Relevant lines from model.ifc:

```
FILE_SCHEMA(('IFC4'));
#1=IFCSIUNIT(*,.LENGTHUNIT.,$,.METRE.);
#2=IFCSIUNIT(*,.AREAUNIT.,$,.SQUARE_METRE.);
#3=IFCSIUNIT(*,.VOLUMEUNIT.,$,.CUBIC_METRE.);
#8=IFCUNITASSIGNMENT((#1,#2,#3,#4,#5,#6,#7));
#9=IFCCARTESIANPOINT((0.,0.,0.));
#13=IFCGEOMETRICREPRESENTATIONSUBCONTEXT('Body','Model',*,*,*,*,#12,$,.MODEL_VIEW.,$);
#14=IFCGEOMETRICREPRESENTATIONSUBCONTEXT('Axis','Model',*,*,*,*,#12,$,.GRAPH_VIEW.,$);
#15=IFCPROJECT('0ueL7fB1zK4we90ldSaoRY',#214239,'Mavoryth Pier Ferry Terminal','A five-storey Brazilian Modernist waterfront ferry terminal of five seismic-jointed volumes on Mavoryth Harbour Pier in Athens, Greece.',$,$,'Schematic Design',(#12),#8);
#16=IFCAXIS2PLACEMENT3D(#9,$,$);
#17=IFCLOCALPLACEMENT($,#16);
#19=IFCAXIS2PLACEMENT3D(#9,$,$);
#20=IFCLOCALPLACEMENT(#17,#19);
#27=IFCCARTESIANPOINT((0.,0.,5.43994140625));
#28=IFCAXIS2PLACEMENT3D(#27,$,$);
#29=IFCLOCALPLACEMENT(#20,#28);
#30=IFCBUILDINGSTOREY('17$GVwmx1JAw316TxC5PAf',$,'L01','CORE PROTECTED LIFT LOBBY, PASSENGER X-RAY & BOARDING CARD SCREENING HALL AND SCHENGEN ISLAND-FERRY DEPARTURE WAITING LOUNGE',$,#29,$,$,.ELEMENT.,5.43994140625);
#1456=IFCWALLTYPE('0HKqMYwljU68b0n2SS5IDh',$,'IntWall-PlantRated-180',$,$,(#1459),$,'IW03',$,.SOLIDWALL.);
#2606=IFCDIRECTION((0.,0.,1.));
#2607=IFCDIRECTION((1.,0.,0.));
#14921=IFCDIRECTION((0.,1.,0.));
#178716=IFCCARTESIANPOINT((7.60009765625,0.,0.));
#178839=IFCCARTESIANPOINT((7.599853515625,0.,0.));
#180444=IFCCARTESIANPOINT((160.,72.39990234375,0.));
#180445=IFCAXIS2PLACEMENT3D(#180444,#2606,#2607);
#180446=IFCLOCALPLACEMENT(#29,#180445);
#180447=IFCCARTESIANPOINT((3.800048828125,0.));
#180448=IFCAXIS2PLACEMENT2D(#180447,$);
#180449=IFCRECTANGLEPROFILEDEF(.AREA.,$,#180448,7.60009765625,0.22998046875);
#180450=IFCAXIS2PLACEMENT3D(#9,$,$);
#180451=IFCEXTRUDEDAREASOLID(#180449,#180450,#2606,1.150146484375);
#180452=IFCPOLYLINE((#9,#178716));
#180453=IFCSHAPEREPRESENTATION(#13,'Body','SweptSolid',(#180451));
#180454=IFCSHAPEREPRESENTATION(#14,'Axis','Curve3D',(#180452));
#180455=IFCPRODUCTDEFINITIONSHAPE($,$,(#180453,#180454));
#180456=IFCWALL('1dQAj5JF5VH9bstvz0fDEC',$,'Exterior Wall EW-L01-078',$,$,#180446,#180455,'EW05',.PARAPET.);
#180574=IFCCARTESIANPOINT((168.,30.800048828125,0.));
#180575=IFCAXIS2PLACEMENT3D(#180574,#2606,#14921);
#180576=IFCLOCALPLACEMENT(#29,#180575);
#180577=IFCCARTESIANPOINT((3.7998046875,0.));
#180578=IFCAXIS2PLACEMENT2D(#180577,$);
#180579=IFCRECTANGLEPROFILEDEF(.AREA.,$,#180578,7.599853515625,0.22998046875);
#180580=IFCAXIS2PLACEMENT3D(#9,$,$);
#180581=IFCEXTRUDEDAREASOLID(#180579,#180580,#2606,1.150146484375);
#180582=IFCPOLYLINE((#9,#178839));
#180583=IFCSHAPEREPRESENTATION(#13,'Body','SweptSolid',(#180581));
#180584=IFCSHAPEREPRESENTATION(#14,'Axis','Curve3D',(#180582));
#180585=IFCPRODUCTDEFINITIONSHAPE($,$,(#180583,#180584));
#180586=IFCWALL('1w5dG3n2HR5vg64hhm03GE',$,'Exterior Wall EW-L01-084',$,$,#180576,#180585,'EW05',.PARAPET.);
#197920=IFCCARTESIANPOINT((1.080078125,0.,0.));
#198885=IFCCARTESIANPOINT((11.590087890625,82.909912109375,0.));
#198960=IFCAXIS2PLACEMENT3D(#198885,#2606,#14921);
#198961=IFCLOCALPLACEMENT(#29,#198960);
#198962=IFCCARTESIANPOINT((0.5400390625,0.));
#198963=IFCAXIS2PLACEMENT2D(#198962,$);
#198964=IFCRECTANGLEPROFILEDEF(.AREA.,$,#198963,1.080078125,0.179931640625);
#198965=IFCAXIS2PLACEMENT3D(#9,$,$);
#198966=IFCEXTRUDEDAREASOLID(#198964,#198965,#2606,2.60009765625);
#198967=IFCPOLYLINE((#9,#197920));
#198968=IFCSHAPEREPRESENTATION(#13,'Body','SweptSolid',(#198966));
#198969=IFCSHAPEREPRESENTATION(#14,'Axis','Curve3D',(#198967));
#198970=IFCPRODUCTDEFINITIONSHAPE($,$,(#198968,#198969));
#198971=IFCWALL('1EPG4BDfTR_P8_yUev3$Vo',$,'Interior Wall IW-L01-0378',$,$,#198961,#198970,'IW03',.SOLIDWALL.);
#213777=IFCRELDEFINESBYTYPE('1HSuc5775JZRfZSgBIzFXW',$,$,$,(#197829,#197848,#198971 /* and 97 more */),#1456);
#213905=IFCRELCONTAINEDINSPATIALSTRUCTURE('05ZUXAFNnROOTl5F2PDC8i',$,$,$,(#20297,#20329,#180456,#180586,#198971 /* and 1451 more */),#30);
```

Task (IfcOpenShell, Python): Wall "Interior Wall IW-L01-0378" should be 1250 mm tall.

```python
import ifcopenshell
import ifcopenshell.geom
import ifcopenshell.util.representation
import ifcopenshell.util.shape

model = ifcopenshell.open("model.ifc")
settings = ifcopenshell.geom.settings()


def volume(element):
    """Net volume in cubic metres, openings subtracted."""
    shape = ifcopenshell.geom.create_shape(settings, element)
    return ifcopenshell.util.shape.get_volume(shape.geometry)


wall = model.by_guid("1EPG4BDfTR_P8_yUev3$Vo")
before = volume(wall)

body = ifcopenshell.util.representation.get_representation(wall, "Model", "Body")
solid = body.Items[0]
old_height = solid.Depth
solid.Depth = 1.25
after = volume(wall)

print(f"height {old_height:g} -> {solid.Depth:g}, volume {before:.3f} -> {after:.3f} m3")

model.write("model_v2.ifc")
```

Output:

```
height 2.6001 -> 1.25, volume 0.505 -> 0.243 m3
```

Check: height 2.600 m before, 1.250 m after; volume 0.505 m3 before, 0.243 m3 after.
